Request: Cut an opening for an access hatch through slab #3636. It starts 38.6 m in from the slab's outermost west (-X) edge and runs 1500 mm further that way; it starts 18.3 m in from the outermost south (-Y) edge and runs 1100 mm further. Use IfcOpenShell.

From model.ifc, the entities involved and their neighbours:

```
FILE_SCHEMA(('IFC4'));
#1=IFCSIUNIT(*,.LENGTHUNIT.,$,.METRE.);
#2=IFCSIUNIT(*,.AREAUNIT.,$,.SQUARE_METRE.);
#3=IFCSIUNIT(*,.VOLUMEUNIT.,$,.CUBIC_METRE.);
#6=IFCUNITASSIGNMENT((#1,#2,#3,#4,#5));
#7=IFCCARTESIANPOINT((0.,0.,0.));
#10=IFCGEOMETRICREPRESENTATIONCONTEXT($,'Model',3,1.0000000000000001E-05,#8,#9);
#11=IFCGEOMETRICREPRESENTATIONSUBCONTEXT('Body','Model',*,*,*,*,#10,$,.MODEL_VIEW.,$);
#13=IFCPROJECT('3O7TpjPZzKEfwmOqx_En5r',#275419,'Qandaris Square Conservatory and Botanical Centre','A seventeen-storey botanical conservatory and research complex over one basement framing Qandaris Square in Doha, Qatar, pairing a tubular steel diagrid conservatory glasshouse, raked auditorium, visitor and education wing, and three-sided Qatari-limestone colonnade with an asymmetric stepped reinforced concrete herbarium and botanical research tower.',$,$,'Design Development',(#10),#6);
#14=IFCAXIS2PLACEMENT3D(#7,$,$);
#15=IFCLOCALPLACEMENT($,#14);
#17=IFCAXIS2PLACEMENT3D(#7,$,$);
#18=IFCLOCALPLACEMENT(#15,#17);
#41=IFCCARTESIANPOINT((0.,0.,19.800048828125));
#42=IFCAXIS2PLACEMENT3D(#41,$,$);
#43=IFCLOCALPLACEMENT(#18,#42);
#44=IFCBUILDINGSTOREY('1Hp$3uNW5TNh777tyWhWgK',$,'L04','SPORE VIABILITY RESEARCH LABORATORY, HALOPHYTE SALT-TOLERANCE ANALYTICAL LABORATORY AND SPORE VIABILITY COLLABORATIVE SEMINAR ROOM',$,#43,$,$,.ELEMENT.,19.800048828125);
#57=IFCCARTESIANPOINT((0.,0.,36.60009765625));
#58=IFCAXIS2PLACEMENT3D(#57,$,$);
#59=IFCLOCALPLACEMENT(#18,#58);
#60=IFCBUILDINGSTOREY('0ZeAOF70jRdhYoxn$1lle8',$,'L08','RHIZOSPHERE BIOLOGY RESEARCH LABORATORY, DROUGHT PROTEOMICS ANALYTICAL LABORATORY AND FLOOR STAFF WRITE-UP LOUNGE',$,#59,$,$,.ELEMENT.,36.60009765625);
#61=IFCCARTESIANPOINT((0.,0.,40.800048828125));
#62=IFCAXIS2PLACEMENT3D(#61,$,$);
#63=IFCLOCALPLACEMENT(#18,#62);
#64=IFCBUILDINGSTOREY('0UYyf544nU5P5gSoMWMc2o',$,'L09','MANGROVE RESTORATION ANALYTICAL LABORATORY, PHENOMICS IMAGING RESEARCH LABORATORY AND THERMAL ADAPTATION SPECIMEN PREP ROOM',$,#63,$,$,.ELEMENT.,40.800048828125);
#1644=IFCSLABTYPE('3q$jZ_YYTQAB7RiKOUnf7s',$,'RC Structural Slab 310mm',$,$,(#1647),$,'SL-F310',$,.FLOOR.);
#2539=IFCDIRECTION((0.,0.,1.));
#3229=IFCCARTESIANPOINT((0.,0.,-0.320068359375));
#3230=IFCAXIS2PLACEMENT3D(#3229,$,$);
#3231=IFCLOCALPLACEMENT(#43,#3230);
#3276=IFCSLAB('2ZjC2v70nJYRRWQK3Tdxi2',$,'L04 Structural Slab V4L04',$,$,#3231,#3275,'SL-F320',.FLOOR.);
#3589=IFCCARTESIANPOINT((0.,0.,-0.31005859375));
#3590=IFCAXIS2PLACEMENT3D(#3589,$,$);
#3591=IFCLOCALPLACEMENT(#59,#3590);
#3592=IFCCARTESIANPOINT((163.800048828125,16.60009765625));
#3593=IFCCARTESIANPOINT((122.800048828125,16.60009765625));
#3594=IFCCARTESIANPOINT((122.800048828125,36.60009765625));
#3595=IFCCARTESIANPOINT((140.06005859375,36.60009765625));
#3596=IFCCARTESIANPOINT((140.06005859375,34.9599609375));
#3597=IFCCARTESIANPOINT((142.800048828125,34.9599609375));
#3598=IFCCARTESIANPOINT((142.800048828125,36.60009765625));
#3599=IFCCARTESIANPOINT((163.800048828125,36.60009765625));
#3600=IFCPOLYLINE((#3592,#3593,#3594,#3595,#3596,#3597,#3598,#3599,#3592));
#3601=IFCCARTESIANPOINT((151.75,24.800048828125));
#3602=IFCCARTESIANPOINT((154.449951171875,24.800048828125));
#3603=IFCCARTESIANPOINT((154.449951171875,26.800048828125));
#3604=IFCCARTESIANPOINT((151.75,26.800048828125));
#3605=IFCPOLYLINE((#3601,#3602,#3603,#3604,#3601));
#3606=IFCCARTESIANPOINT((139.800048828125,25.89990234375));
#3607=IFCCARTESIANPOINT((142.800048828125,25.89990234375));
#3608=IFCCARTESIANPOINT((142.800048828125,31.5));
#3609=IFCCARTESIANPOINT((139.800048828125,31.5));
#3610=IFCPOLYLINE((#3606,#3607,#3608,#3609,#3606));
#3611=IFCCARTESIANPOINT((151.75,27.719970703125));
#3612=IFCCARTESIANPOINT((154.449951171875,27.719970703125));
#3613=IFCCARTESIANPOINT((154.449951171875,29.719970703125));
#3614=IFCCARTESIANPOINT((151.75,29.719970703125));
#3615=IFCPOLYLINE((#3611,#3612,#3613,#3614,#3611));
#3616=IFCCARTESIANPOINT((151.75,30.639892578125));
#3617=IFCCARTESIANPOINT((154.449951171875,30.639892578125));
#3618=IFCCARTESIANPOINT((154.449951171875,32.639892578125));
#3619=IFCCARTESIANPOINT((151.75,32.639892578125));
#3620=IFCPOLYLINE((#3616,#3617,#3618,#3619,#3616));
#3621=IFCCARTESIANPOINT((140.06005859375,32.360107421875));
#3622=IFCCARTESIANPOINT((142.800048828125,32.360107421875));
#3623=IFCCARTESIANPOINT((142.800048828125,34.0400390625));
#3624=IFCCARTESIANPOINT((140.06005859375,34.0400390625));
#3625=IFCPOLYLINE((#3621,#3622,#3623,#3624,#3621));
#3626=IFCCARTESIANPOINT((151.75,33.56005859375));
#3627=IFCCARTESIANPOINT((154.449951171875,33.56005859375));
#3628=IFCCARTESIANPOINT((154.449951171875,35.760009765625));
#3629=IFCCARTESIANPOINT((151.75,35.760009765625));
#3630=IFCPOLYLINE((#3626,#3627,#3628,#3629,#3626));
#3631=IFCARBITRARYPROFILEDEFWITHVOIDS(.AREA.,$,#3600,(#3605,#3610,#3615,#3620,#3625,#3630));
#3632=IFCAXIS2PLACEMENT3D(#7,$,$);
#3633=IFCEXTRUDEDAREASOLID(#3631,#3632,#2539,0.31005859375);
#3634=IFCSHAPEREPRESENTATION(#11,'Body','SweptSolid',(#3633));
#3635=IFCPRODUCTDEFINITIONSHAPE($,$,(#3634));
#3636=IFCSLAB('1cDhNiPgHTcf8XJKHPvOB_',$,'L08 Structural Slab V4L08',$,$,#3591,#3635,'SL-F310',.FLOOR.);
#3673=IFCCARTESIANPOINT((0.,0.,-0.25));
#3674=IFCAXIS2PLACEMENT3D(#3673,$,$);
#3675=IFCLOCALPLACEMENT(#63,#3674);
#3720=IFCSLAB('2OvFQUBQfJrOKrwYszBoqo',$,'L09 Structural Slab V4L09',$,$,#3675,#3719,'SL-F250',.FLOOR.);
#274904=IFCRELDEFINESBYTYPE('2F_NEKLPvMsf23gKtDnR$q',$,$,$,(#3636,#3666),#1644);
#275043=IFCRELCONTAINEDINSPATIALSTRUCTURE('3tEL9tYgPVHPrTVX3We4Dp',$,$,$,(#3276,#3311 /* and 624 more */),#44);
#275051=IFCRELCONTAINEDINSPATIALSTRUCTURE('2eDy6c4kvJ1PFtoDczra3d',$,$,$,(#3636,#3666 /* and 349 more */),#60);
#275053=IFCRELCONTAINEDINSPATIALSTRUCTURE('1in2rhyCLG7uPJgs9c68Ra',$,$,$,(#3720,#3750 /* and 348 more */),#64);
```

```python
import numpy as np
import ifcopenshell
import ifcopenshell.api.feature
import ifcopenshell.api.geometry
import ifcopenshell.api.root
import ifcopenshell.geom
import ifcopenshell.util.placement
import ifcopenshell.util.representation
import ifcopenshell.util.shape
import ifcopenshell.util.unit

model = ifcopenshell.open("model.ifc")
unit_scale = ifcopenshell.util.unit.calculate_unit_scale(model)
settings = ifcopenshell.geom.settings()


def volume(element):
    """Net volume in cubic metres, openings subtracted."""
    shape = ifcopenshell.geom.create_shape(settings, element)
    return ifcopenshell.util.shape.get_volume(shape.geometry)


slab = model.by_guid("1cDhNiPgHTcf8XJKHPvOB_")
before = volume(slab)

# Extent in the slab's own axes, in metres. The edges named are its -X and -Y sides.
slab_shape = ifcopenshell.geom.create_shape(settings, slab)
vertices = ifcopenshell.util.shape.get_vertices(slab_shape.geometry)
x_min, y_min, bottom = vertices.min(axis=0)
top = vertices[:, 2].max()

opening = ifcopenshell.api.root.create_entity(model, ifc_class="IfcOpeningElement", name="Access hatch opening", predefined_type="OPENING")
context = ifcopenshell.util.representation.get_context(model, "Model", "Body", "MODEL_VIEW")
width, depth = 1.5, 1.1
outline = [(0.0, 0.0), (width, 0.0), (width, depth), (0.0, depth), (0.0, 0.0)]
# Overshoot both faces by 50 mm so the cut is clean.
shape = ifcopenshell.api.geometry.add_slab_representation(
    model, context=context, depth=top - bottom + 0.1, polyline=outline
)
ifcopenshell.api.geometry.assign_representation(model, product=opening, representation=shape)

matrix = ifcopenshell.util.placement.get_local_placement(slab.ObjectPlacement)
matrix[:, 3] = matrix @ np.append(np.array([x_min + 38.6, y_min + 18.3, bottom - 0.05]) / unit_scale, 1.0)
ifcopenshell.api.geometry.edit_object_placement(model, product=opening, matrix=matrix, is_si=False)
ifcopenshell.api.feature.add_feature(model, feature=opening, element=slab)

after = volume(slab)

print(f"slab volume {before:.3f} -> {after:.3f} m3")

model.write("model_v2.ifc")
```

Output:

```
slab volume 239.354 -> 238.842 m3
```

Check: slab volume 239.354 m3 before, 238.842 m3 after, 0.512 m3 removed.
